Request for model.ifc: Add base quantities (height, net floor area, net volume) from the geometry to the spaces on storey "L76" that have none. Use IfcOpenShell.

First a look at what the model holds.

```python
import ifcopenshell
import ifcopenshell.util.element
import ifcopenshell.util.unit

model = ifcopenshell.open("model.ifc")
print(model.schema)
for unit_type in ("LENGTHUNIT", "AREAUNIT", "VOLUMEUNIT"):
    print(unit_type, ifcopenshell.util.unit.calculate_unit_scale(model, unit_type))
storey = next(s for s in model.by_type("IfcBuildingStorey") if s.Name == "L76")
spaces = [e for e in ifcopenshell.util.element.get_decomposition(storey) if e.is_a("IfcSpace")]
for e in sorted(spaces, key=lambda e: e.id()):
    print(e.id(), e.is_a(), e.Name, list(ifcopenshell.util.element.get_psets(e, qtos_only=True)), sep=" | ")
```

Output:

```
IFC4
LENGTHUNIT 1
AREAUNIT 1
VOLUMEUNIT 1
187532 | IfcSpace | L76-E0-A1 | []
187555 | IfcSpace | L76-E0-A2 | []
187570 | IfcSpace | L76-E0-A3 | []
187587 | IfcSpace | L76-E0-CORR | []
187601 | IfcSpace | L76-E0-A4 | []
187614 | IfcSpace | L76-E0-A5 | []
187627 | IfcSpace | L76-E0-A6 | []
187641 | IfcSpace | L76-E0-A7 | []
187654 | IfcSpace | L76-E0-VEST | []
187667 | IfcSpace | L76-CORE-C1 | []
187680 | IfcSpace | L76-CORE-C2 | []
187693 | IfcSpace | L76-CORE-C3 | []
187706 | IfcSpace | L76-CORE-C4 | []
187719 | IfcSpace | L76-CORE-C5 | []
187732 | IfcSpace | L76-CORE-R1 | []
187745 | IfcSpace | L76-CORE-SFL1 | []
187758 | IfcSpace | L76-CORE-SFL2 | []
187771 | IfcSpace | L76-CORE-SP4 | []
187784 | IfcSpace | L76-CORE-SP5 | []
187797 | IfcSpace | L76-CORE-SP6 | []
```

```python
import ifcopenshell
import ifcopenshell.api.pset
import ifcopenshell.geom
import ifcopenshell.util.element
import ifcopenshell.util.shape
import ifcopenshell.util.unit

model = ifcopenshell.open("model.ifc")
unit_scale = ifcopenshell.util.unit.calculate_unit_scale(model)
area_scale = ifcopenshell.util.unit.calculate_unit_scale(model, "AREAUNIT")
volume_scale = ifcopenshell.util.unit.calculate_unit_scale(model, "VOLUMEUNIT")
settings = ifcopenshell.geom.settings()

storey = next(s for s in model.by_type("IfcBuildingStorey") if s.Name == "L76")
spaces = [e for e in ifcopenshell.util.element.get_decomposition(storey) if e.is_a("IfcSpace")]

for e in sorted(spaces, key=lambda e: e.id()):
    if ifcopenshell.util.element.get_psets(e, qtos_only=True, should_inherit=False):
        continue
    # Geometry comes back in metres, in the element's own axes.
    shape = ifcopenshell.geom.create_shape(settings, e)
    values = {
        "Height": ifcopenshell.util.shape.get_z(shape.geometry) / unit_scale,
        "NetFloorArea": ifcopenshell.util.shape.get_footprint_area(shape.geometry) / area_scale,
        "NetVolume": ifcopenshell.util.shape.get_volume(shape.geometry) / volume_scale,
    }
    qto = ifcopenshell.api.pset.add_qto(model, product=e, name="Qto_SpaceBaseQuantities")
    ifcopenshell.api.pset.edit_qto(model, qto=qto, properties=values)
    print(e.id(), {k: round(v, 3) for k, v in values.items()})

model.write("model-out.ifc")
```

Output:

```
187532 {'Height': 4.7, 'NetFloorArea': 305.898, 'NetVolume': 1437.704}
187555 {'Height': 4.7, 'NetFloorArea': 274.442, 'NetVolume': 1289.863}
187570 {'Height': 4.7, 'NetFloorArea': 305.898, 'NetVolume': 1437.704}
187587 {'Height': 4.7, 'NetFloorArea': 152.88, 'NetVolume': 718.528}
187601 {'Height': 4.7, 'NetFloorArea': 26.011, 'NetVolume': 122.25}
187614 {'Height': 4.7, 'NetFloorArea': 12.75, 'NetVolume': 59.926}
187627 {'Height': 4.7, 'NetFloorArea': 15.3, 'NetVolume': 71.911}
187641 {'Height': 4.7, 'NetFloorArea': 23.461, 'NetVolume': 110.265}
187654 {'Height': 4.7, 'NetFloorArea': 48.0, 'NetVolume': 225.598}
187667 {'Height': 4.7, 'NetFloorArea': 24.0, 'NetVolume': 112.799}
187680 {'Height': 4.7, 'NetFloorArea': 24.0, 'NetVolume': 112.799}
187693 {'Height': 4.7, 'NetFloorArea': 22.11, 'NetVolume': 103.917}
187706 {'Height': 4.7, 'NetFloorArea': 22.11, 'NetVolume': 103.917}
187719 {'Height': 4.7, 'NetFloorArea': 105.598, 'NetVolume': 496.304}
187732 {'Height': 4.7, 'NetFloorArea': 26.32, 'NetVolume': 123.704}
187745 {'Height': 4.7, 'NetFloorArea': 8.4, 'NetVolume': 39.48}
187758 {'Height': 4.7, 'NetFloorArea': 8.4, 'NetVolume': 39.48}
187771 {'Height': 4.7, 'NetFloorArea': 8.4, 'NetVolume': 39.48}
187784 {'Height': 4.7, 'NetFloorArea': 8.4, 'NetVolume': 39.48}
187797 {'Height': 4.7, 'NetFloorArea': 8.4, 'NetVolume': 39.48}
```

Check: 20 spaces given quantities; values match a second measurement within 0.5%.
